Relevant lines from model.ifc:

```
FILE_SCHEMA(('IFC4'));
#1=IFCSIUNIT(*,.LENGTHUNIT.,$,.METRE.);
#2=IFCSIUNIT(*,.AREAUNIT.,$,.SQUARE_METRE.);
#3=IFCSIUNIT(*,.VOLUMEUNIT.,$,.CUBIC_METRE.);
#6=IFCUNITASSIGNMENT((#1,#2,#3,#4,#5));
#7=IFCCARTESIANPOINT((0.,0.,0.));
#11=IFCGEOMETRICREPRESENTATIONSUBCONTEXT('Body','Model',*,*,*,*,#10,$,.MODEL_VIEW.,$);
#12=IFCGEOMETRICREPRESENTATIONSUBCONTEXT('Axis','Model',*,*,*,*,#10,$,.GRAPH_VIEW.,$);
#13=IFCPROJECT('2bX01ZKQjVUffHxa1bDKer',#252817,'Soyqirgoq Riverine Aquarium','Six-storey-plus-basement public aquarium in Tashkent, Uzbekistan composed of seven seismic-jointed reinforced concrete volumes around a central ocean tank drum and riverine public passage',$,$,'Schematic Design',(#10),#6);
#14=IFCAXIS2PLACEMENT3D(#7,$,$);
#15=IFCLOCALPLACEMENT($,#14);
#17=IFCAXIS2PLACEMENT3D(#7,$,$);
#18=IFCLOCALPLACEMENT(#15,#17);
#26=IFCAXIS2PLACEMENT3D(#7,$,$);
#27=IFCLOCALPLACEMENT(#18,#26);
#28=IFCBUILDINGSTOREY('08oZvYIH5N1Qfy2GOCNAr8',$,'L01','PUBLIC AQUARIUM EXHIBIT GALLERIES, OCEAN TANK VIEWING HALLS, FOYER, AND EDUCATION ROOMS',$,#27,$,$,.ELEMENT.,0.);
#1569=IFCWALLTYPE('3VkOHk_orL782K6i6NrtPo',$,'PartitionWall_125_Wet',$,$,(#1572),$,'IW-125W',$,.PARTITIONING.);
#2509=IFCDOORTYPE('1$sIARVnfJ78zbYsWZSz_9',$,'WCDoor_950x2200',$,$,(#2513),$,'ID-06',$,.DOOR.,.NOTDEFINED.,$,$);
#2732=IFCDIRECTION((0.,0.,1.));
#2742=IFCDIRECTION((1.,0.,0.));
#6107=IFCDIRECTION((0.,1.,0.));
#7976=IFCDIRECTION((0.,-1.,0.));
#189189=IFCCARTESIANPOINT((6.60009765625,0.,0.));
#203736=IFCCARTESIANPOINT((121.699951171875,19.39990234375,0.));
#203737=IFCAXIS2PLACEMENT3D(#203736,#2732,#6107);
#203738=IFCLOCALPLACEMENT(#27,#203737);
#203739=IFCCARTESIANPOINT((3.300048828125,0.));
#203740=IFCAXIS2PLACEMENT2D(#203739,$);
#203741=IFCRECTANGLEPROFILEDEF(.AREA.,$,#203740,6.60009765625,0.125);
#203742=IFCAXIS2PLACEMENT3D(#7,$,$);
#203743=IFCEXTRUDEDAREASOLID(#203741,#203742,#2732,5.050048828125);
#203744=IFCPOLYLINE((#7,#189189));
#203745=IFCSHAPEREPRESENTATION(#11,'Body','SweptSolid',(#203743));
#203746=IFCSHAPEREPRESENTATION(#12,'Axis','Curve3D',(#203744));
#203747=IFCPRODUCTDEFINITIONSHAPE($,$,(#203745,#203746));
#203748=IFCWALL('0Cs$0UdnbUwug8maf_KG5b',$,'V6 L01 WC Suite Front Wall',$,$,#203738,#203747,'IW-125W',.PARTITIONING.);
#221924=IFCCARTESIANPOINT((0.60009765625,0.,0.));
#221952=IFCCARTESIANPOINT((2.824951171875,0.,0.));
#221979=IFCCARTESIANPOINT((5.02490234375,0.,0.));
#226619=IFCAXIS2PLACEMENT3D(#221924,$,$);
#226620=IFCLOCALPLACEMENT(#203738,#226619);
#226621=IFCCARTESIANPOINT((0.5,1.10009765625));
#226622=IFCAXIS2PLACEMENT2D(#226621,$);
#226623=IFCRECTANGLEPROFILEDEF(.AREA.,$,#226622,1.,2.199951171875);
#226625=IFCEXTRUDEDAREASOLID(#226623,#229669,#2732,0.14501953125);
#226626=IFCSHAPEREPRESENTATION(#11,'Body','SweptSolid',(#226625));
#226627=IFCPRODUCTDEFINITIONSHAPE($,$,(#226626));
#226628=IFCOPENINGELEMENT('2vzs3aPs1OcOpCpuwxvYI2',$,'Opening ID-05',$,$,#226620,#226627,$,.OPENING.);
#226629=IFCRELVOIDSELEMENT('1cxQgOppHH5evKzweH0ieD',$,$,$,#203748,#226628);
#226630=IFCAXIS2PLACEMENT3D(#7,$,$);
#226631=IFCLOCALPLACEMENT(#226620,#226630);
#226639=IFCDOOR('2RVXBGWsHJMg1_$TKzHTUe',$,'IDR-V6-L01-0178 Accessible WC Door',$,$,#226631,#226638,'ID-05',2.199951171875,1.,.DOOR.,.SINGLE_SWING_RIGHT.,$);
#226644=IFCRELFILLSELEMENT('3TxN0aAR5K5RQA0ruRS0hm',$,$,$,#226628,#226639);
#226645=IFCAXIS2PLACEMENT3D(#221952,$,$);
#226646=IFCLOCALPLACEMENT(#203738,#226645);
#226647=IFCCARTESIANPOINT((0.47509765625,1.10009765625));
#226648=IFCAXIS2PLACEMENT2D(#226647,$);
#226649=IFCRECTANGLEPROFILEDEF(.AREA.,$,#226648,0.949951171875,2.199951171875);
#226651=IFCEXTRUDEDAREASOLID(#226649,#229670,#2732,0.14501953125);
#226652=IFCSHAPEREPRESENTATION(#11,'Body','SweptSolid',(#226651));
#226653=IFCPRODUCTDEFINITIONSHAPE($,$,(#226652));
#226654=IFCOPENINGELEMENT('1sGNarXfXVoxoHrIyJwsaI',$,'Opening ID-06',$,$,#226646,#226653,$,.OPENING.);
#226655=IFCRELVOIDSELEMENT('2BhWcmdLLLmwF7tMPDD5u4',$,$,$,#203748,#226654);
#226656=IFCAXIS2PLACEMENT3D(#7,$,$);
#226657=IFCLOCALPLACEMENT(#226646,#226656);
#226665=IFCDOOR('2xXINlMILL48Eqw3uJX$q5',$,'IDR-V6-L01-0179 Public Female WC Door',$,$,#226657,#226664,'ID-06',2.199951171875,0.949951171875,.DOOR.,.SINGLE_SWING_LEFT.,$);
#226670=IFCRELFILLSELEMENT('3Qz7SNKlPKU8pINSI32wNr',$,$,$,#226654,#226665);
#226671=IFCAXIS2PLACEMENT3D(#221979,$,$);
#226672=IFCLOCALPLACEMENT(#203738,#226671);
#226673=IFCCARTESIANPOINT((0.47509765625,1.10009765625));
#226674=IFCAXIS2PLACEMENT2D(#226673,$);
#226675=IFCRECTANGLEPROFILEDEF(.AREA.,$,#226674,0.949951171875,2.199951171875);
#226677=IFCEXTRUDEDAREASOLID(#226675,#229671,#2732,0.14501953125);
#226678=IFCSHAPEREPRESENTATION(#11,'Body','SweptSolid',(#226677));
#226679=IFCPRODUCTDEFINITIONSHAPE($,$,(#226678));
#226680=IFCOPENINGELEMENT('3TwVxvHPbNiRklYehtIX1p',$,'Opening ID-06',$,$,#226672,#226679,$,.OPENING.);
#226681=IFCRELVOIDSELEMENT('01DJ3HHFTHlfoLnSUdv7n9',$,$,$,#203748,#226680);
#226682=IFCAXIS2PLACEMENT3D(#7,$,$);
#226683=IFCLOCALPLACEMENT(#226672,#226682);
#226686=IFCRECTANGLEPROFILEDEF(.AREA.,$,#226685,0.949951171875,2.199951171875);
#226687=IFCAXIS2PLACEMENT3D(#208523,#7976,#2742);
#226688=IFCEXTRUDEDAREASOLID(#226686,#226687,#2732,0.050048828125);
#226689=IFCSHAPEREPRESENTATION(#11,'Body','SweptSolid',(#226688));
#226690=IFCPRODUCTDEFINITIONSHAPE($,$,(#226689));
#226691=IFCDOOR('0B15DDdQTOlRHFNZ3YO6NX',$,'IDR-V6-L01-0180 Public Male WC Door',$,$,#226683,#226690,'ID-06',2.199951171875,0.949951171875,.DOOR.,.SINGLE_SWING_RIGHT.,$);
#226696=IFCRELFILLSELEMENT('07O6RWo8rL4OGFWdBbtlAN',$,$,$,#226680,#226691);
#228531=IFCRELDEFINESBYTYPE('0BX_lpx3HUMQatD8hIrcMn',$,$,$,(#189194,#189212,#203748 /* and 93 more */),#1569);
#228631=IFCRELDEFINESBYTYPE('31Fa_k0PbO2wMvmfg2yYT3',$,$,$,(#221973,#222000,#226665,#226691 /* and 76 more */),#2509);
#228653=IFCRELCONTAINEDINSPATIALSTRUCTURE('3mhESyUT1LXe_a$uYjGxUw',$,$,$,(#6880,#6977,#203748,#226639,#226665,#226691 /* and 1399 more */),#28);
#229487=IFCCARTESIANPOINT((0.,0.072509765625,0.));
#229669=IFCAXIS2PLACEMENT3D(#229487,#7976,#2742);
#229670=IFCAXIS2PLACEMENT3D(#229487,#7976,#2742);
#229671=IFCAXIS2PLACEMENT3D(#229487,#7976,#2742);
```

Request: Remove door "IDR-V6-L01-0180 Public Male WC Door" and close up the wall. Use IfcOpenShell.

```python
import ifcopenshell
import ifcopenshell.api.feature
import ifcopenshell.api.root
import ifcopenshell.geom
import ifcopenshell.util.shape

model = ifcopenshell.open("model.ifc")
settings = ifcopenshell.geom.settings()


def volume(element):
    """Net volume in cubic metres, openings subtracted."""
    shape = ifcopenshell.geom.create_shape(settings, element)
    return ifcopenshell.util.shape.get_volume(shape.geometry)


door = model.by_id(226691)
opening = door.FillsVoids[0].RelatingOpeningElement
wall = opening.VoidsElements[0].RelatingBuildingElement
before = volume(wall)

ifcopenshell.api.root.remove_product(model, product=door)
ifcopenshell.api.feature.remove_feature(model, feature=opening)

after = volume(wall)

print(f"wall volume {before:.3f} -> {after:.3f} m3")

model.write("model_updated.ifc")
```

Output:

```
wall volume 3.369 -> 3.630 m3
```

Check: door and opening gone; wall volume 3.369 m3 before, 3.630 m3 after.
